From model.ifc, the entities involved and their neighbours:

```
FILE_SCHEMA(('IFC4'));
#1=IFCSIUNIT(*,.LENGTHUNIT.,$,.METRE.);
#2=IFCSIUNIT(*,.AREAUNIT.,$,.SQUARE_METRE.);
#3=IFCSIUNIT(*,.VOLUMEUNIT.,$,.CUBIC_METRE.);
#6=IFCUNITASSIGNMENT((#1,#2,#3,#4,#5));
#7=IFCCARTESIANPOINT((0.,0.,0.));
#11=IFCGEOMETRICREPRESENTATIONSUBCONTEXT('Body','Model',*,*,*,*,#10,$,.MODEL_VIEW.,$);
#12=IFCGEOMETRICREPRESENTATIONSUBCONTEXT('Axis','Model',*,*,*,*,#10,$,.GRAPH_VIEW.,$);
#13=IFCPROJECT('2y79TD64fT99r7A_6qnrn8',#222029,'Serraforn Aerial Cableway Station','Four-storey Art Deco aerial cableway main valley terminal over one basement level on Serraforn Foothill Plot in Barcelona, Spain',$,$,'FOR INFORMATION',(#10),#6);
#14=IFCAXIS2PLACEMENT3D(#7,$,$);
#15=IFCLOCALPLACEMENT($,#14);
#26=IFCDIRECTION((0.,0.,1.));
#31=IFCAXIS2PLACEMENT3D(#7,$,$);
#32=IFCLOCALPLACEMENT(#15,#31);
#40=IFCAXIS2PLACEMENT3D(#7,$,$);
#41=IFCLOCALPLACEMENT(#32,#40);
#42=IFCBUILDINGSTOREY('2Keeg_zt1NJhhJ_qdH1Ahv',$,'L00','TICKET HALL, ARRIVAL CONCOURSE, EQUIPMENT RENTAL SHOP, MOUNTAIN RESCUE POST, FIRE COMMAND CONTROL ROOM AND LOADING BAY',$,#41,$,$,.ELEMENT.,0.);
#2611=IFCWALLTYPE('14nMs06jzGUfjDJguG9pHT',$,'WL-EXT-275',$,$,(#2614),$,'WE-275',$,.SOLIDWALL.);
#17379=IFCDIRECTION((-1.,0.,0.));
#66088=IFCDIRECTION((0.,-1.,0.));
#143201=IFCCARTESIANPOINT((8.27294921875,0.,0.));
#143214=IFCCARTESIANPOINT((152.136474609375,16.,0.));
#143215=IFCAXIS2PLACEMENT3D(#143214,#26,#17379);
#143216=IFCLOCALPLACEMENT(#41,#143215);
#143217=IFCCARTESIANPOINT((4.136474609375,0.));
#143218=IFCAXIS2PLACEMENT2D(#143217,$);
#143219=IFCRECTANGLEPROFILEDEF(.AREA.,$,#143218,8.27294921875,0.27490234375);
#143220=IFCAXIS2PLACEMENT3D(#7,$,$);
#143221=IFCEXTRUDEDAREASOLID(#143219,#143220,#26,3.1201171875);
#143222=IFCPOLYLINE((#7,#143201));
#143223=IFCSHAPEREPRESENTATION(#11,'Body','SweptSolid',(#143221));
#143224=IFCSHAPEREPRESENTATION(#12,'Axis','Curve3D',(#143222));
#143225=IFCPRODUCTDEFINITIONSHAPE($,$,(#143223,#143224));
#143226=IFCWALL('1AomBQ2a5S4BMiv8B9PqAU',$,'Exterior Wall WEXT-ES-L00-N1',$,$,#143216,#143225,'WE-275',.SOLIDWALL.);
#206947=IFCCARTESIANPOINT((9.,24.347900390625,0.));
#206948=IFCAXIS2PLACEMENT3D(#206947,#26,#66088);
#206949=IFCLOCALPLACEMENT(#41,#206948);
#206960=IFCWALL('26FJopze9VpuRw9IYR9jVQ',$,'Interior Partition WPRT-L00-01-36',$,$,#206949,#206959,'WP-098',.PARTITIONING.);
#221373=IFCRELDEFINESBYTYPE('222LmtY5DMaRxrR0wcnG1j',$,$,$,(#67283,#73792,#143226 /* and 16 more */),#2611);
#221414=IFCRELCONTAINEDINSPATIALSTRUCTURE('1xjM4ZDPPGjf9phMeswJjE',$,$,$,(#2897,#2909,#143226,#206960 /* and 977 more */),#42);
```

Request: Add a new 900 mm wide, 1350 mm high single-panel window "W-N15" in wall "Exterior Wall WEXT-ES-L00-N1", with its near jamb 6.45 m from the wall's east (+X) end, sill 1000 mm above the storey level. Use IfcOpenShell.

```python
import numpy as np
import ifcopenshell
import ifcopenshell.api.feature
import ifcopenshell.api.geometry
import ifcopenshell.api.root
import ifcopenshell.api.spatial
import ifcopenshell.geom
import ifcopenshell.util.element
import ifcopenshell.util.placement
import ifcopenshell.util.representation
import ifcopenshell.util.shape
import ifcopenshell.util.unit

model = ifcopenshell.open("model.ifc")
unit_scale = ifcopenshell.util.unit.calculate_unit_scale(model)
settings = ifcopenshell.geom.settings()


def volume(element):
    """Net volume in cubic metres, openings subtracted."""
    shape = ifcopenshell.geom.create_shape(settings, element)
    return ifcopenshell.util.shape.get_volume(shape.geometry)


wall = model.by_guid("1AomBQ2a5S4BMiv8B9PqAU")
storey = ifcopenshell.util.element.get_container(wall, ifc_class="IfcBuildingStorey")
context = ifcopenshell.util.representation.get_context(model, "Model", "Body", "MODEL_VIEW")
before = volume(wall)

width, height, from_end, sill = 0.9, 1.35, 6.45, 1  # metres

# The wall runs along its own X axis, and the end named is its -X end.
wall_shape = ifcopenshell.geom.create_shape(settings, wall)
x, y, z = ifcopenshell.util.shape.get_vertices(wall_shape.geometry).T
start = x.min() + from_end
face, thickness = float(y.min()), float(y.max() - y.min())
wall_matrix = ifcopenshell.util.placement.get_local_placement(wall.ObjectPlacement)
level = ifcopenshell.util.placement.get_local_placement(storey.ObjectPlacement)[2, 3]


def in_wall(x, y):
    """Placement at x, y metres in the wall's axes, at sill height."""
    matrix = wall_matrix.copy()
    matrix[:, 3] = wall_matrix @ np.array([x / unit_scale, y / unit_scale, 0.0, 1.0])
    matrix[2, 3] = level + sill / unit_scale
    return matrix


# Opening: a box that overshoots both wall faces by 50 mm.
opening = ifcopenshell.api.root.create_entity(model, ifc_class="IfcOpeningElement", predefined_type="OPENING")
box = ifcopenshell.api.geometry.add_wall_representation(
    model, context=context, length=width, height=height, thickness=thickness + 0.1
)
ifcopenshell.api.geometry.assign_representation(model, product=opening, representation=box)
ifcopenshell.api.geometry.edit_object_placement(model, product=opening, matrix=in_wall(start, face - 0.05), is_si=False)
ifcopenshell.api.feature.add_feature(model, feature=opening, element=wall)

window = ifcopenshell.api.root.create_entity(model, ifc_class="IfcWindow", name="W-N15", predefined_type="WINDOW")
window.OverallWidth, window.OverallHeight = width / unit_scale, height / unit_scale
window.PartitioningType = "SINGLE_PANEL"
body = ifcopenshell.api.geometry.add_window_representation(
    model,
    context=context,
    overall_width=window.OverallWidth,
    overall_height=window.OverallHeight,
    partition_type="SINGLE_PANEL",
)
ifcopenshell.api.geometry.assign_representation(model, product=window, representation=body)
ifcopenshell.api.spatial.assign_container(model, products=[window], relating_structure=storey)
ifcopenshell.api.feature.add_filling(model, opening=opening, element=window)

# Centre the window in the wall's thickness.
ifcopenshell.api.geometry.edit_object_placement(model, product=window, matrix=in_wall(start, face), is_si=False)
window_shape = ifcopenshell.geom.create_shape(settings, window)
depth = ifcopenshell.util.shape.get_vertices(window_shape.geometry)[:, 1]
offset = face + thickness / 2 - (depth.min() + depth.max()) / 2
ifcopenshell.api.geometry.edit_object_placement(model, product=window, matrix=in_wall(start, offset), is_si=False)

after = volume(wall)

print(f"wall volume {before:.3f} -> {after:.3f} m3")

model.write("model_v2.ifc")
```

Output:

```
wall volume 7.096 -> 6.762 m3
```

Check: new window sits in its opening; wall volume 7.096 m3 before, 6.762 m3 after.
